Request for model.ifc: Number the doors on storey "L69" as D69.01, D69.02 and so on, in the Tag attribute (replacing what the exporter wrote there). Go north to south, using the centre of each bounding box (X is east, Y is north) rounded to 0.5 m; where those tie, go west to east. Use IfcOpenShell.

First a look at what the model holds.

```python
import ifcopenshell
import ifcopenshell.util.element
import ifcopenshell.util.placement

model = ifcopenshell.open("model.ifc")
print(model.schema)
storey = next(s for s in model.by_type("IfcBuildingStorey") if s.Name == "L69")
doors = [e for e in ifcopenshell.util.element.get_decomposition(storey) if e.is_a("IfcDoor")]
for e in sorted(doors, key=lambda e: e.id()):
    origin = ifcopenshell.util.placement.get_local_placement(e.ObjectPlacement)[:3, 3]
    print(e.id(), e.Tag, e.Name, origin.round(2) + 0.0, sep=" | ")
```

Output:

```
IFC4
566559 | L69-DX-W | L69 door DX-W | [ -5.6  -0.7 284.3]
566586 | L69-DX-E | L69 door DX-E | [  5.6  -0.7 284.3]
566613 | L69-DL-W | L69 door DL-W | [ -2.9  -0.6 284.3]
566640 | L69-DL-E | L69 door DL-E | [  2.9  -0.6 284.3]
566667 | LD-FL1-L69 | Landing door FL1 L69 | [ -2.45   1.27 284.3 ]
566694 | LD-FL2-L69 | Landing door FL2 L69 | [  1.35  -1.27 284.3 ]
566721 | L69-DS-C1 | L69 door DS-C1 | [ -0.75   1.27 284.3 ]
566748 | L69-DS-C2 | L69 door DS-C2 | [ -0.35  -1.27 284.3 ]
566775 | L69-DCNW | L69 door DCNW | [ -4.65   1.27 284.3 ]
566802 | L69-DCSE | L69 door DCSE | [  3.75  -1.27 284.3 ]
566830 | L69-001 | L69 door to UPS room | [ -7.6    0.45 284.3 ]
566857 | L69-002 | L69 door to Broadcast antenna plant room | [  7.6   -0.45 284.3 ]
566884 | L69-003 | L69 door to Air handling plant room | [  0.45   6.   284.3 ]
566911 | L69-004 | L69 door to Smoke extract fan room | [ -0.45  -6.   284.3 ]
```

```python
import ifcopenshell
import ifcopenshell.geom
import ifcopenshell.util.element
import ifcopenshell.util.shape

model = ifcopenshell.open("model.ifc")
settings = ifcopenshell.geom.settings()
settings.set("use-world-coords", True)


def centre(element):
    shape = ifcopenshell.geom.create_shape(settings, element)
    return ifcopenshell.util.shape.get_bbox_centroid(shape.geometry)


storey = next(s for s in model.by_type("IfcBuildingStorey") if s.Name == "L69")
doors = [e for e in ifcopenshell.util.element.get_decomposition(storey) if e.is_a("IfcDoor")]

# Insertion points can sit at a corner or the storey origin, so sort by the geometry (in metres).
centres = {e: centre(e) for e in doors}
doors.sort(key=lambda e: (-round(centres[e][1] / 0.5), centres[e][0]))

for i, e in enumerate(doors, start=1):
    number = f"D69.{i:02d}"
    e.Tag = number
    print(e.id(), number)

model.write("model_v2.ifc")
```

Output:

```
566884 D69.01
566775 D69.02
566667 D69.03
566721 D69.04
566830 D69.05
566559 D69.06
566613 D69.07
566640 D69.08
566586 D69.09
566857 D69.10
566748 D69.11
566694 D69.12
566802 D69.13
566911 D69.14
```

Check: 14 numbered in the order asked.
